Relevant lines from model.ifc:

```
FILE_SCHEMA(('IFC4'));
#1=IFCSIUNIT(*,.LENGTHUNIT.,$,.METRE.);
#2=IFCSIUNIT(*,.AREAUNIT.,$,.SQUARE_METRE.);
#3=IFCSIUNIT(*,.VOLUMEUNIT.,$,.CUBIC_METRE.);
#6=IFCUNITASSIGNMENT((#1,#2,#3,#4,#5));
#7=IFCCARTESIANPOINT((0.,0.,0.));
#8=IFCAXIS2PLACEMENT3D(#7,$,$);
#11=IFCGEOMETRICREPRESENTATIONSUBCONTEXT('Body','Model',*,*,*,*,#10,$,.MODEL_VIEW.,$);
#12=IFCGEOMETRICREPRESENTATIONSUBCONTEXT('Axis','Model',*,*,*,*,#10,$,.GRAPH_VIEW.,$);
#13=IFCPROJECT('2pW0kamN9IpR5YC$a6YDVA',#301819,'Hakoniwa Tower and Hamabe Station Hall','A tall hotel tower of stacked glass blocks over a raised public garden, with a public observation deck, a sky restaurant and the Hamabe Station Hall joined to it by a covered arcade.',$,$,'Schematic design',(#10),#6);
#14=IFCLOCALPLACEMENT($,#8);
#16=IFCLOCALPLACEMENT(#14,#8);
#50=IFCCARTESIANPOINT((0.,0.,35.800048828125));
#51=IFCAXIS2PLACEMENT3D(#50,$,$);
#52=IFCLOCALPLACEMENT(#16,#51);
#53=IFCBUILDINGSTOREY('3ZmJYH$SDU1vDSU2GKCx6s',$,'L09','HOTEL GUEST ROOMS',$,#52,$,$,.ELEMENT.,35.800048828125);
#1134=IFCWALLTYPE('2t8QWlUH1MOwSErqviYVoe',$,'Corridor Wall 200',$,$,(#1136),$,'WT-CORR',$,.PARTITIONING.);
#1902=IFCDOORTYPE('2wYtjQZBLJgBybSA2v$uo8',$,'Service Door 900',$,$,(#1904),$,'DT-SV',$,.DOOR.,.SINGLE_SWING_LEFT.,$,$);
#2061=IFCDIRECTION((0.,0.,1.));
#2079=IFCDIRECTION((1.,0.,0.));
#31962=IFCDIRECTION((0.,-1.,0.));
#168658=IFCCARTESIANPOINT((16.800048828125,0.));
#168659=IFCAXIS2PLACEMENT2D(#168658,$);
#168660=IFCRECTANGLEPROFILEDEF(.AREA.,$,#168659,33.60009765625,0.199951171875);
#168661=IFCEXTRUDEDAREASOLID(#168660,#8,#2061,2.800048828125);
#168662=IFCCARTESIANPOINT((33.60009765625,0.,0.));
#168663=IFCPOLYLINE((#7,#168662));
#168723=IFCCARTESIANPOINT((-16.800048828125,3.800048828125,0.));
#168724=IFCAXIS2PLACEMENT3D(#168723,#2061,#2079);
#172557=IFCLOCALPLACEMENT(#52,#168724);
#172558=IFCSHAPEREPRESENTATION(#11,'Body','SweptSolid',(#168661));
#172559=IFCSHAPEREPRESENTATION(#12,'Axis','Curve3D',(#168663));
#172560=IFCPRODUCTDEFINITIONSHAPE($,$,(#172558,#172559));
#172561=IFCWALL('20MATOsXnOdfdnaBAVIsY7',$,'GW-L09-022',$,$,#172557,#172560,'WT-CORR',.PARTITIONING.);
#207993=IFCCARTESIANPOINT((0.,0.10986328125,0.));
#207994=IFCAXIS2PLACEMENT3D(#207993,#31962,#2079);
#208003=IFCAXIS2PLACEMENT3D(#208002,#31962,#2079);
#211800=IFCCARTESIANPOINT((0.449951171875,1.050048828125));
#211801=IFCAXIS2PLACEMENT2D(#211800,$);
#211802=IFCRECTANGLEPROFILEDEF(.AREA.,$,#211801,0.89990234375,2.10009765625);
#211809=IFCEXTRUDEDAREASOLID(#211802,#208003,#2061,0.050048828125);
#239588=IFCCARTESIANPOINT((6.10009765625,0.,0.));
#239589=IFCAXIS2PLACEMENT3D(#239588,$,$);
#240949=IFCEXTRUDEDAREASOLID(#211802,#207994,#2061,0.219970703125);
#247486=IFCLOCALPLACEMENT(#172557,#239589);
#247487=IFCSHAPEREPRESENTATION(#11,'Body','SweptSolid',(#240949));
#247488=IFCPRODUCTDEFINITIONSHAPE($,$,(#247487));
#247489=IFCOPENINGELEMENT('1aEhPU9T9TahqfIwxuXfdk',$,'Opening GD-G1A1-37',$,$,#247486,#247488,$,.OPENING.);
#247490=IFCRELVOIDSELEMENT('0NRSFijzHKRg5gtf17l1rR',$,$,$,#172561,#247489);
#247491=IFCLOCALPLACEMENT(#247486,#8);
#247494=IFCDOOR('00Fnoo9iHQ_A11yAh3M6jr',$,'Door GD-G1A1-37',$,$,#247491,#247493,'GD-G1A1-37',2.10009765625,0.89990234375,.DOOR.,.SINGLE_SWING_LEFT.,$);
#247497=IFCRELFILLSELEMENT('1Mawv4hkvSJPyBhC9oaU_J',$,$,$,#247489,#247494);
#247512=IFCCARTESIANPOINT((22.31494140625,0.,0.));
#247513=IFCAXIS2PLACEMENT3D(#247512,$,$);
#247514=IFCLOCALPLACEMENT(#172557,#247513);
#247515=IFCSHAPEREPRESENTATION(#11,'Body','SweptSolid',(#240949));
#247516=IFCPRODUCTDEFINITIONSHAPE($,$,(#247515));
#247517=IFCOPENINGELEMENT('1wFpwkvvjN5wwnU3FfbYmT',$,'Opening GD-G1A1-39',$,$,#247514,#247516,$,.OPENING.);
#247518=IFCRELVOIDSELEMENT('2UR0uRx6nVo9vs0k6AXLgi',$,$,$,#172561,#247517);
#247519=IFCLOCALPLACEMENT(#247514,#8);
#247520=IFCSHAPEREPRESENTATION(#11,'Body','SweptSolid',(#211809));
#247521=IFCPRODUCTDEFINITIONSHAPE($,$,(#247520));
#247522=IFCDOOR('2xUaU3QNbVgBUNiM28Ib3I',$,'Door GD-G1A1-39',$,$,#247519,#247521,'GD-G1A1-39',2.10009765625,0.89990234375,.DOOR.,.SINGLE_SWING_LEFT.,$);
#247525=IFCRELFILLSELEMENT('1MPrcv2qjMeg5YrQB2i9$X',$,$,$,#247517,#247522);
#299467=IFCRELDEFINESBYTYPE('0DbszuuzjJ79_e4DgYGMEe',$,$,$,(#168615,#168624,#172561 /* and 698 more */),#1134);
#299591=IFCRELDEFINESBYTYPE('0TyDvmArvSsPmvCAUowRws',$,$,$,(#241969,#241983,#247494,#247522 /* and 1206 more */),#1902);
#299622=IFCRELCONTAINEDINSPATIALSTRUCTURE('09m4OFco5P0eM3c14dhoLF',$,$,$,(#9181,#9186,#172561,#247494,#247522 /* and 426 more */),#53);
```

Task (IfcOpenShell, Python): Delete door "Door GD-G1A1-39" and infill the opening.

```python
import ifcopenshell
import ifcopenshell.api.feature
import ifcopenshell.api.root
import ifcopenshell.geom
import ifcopenshell.util.shape

model = ifcopenshell.open("model.ifc")
settings = ifcopenshell.geom.settings()


def volume(element):
    """Net volume in cubic metres, openings subtracted."""
    shape = ifcopenshell.geom.create_shape(settings, element)
    return ifcopenshell.util.shape.get_volume(shape.geometry)


door = model.by_guid("2xUaU3QNbVgBUNiM28Ib3I")
opening = door.FillsVoids[0].RelatingOpeningElement
wall = opening.VoidsElements[0].RelatingBuildingElement
before = volume(wall)

ifcopenshell.api.root.remove_product(model, product=door)
ifcopenshell.api.feature.remove_feature(model, feature=opening)

after = volume(wall)

print(f"wall volume {before:.3f} -> {after:.3f} m3")

model.write("model_updated.ifc")
```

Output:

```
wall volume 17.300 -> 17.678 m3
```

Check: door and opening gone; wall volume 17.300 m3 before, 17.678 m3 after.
